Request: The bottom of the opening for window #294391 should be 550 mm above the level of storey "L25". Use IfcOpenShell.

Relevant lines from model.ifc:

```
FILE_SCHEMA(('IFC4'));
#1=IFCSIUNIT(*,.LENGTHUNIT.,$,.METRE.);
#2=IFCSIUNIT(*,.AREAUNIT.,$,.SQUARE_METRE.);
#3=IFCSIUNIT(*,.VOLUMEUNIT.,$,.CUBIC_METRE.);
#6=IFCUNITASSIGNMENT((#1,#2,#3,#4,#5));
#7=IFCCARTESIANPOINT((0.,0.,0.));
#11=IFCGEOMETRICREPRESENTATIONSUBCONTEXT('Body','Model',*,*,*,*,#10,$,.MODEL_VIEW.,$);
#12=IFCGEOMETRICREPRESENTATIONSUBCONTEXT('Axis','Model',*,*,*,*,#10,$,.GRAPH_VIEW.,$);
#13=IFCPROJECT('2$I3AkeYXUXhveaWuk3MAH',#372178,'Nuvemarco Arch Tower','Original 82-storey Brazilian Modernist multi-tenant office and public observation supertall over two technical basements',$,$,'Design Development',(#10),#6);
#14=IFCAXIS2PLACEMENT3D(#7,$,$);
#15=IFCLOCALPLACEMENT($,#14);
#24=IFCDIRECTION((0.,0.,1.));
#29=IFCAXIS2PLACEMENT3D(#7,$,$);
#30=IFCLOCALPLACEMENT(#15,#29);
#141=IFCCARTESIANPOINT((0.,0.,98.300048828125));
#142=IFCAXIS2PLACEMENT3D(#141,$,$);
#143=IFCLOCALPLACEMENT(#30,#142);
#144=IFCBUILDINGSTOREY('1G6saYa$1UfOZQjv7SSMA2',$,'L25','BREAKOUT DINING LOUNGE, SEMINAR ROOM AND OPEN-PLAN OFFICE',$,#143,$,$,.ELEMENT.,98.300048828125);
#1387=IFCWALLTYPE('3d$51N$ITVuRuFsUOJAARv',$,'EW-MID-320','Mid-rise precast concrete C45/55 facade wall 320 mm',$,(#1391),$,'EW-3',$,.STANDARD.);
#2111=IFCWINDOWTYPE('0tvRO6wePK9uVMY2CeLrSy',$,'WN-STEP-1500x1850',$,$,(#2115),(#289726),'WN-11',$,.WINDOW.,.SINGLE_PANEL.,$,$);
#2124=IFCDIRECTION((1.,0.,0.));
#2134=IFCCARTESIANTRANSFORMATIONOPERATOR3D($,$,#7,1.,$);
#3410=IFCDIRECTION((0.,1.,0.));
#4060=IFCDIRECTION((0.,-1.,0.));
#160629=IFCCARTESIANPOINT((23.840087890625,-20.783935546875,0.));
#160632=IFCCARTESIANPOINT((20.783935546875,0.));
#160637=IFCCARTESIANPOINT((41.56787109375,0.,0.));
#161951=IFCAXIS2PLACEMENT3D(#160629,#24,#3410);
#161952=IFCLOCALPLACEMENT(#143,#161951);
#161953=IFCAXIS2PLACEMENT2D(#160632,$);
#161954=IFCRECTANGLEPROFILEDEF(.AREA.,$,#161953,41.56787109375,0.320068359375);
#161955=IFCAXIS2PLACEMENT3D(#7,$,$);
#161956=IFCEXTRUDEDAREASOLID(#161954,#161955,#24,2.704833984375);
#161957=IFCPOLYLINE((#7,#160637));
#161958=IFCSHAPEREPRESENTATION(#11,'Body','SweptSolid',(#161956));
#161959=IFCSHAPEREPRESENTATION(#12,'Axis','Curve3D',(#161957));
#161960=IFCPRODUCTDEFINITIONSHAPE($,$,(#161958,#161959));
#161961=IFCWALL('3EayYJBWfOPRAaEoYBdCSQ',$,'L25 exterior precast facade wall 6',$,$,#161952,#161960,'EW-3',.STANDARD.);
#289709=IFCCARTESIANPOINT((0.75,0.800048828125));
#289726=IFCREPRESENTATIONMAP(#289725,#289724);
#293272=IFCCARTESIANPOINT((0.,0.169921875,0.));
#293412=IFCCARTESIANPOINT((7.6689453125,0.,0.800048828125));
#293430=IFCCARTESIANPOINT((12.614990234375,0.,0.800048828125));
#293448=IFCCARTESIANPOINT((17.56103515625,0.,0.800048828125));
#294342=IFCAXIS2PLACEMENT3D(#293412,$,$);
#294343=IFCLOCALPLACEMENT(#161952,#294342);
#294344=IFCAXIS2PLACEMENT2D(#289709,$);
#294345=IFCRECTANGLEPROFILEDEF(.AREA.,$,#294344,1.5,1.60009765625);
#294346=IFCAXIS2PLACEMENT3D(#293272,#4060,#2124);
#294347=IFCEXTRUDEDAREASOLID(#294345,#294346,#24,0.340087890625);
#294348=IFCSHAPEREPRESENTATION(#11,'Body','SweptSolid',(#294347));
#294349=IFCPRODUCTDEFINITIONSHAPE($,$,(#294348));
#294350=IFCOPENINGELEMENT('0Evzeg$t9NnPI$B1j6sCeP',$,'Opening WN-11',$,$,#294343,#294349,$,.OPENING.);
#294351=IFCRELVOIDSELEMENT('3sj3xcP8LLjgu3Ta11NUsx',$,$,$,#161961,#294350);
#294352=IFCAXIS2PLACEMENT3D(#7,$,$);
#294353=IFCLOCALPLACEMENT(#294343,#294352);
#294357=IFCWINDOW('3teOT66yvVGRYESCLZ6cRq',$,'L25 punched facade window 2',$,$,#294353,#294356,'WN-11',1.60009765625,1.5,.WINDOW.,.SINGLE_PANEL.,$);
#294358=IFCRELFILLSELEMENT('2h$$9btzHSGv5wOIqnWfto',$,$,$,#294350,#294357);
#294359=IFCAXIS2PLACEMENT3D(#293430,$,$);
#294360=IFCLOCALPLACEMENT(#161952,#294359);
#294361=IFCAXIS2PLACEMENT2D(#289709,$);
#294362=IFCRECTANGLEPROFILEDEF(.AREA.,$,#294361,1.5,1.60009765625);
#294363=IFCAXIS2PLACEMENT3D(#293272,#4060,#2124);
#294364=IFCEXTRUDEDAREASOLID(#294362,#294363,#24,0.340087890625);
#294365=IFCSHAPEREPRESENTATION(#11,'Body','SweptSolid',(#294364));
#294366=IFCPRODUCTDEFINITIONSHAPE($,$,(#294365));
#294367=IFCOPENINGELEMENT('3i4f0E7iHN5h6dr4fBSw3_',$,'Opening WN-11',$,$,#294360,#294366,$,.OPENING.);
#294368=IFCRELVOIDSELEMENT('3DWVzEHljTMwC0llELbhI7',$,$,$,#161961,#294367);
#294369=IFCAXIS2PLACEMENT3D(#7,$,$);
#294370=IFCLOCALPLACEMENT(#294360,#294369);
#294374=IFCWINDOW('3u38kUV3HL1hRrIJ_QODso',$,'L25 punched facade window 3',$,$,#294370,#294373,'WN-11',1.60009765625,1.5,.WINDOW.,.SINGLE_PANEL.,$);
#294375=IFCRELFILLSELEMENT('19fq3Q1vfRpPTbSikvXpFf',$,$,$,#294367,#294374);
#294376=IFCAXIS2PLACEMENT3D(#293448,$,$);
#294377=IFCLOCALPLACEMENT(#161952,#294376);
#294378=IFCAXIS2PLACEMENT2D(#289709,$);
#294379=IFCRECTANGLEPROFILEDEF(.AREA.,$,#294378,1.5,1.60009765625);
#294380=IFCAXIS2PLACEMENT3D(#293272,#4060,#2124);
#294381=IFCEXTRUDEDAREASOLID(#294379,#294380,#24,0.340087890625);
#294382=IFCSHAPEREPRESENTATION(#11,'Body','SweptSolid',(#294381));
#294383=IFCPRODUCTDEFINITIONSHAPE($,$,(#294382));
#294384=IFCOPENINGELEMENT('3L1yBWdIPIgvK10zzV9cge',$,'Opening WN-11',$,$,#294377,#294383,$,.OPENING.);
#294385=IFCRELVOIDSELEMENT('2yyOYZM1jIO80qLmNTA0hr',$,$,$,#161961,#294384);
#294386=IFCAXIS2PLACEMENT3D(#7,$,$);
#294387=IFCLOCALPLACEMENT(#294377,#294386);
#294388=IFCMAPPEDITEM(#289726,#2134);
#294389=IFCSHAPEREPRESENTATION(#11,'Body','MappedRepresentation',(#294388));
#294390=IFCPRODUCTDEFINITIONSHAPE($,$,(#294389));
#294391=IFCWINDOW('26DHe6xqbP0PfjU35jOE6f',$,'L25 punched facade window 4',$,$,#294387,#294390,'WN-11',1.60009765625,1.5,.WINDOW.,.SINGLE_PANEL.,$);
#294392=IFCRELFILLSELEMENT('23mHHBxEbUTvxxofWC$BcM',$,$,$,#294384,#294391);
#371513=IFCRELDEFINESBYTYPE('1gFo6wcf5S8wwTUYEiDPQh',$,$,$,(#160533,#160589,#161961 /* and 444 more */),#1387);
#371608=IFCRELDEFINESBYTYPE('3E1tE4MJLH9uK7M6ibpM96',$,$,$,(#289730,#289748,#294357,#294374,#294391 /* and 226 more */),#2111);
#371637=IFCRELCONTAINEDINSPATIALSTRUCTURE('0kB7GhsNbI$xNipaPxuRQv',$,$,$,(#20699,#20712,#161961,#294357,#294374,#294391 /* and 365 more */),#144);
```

```python
import numpy as np
import ifcopenshell
import ifcopenshell.api.geometry
import ifcopenshell.geom
import ifcopenshell.util.element
import ifcopenshell.util.placement
import ifcopenshell.util.shape
import ifcopenshell.util.unit

model = ifcopenshell.open("model.ifc")
unit_scale = ifcopenshell.util.unit.calculate_unit_scale(model)

window = model.by_id(294391)
opening = window.FillsVoids[0].RelatingOpeningElement
storey = ifcopenshell.util.element.get_container(window, ifc_class="IfcBuildingStorey")
level = ifcopenshell.util.placement.get_local_placement(storey.ObjectPlacement)[2, 3]

# The opening's origin need not be at the sill, so measure its lowest point.
shape = ifcopenshell.geom.create_shape(ifcopenshell.geom.settings(), opening)
bottom = ifcopenshell.util.shape.get_shape_bottom_elevation(shape, shape.geometry) / unit_scale
dz = level + 0.55 / unit_scale - bottom

shift = np.array([0.0, 0.0, dz])
# The window is placed relative to its opening, so it follows when the opening moves.
matrix = ifcopenshell.util.placement.get_local_placement(opening.ObjectPlacement)
matrix[:3, 3] += shift
ifcopenshell.api.geometry.edit_object_placement(
    model, product=opening, matrix=matrix, is_si=False, should_transform_children=True
)

print(f"moved by {dz * unit_scale:+.3f} m")

model.write("model_rev.ifc")
```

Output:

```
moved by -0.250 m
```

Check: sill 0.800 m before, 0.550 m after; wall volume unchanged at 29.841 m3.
